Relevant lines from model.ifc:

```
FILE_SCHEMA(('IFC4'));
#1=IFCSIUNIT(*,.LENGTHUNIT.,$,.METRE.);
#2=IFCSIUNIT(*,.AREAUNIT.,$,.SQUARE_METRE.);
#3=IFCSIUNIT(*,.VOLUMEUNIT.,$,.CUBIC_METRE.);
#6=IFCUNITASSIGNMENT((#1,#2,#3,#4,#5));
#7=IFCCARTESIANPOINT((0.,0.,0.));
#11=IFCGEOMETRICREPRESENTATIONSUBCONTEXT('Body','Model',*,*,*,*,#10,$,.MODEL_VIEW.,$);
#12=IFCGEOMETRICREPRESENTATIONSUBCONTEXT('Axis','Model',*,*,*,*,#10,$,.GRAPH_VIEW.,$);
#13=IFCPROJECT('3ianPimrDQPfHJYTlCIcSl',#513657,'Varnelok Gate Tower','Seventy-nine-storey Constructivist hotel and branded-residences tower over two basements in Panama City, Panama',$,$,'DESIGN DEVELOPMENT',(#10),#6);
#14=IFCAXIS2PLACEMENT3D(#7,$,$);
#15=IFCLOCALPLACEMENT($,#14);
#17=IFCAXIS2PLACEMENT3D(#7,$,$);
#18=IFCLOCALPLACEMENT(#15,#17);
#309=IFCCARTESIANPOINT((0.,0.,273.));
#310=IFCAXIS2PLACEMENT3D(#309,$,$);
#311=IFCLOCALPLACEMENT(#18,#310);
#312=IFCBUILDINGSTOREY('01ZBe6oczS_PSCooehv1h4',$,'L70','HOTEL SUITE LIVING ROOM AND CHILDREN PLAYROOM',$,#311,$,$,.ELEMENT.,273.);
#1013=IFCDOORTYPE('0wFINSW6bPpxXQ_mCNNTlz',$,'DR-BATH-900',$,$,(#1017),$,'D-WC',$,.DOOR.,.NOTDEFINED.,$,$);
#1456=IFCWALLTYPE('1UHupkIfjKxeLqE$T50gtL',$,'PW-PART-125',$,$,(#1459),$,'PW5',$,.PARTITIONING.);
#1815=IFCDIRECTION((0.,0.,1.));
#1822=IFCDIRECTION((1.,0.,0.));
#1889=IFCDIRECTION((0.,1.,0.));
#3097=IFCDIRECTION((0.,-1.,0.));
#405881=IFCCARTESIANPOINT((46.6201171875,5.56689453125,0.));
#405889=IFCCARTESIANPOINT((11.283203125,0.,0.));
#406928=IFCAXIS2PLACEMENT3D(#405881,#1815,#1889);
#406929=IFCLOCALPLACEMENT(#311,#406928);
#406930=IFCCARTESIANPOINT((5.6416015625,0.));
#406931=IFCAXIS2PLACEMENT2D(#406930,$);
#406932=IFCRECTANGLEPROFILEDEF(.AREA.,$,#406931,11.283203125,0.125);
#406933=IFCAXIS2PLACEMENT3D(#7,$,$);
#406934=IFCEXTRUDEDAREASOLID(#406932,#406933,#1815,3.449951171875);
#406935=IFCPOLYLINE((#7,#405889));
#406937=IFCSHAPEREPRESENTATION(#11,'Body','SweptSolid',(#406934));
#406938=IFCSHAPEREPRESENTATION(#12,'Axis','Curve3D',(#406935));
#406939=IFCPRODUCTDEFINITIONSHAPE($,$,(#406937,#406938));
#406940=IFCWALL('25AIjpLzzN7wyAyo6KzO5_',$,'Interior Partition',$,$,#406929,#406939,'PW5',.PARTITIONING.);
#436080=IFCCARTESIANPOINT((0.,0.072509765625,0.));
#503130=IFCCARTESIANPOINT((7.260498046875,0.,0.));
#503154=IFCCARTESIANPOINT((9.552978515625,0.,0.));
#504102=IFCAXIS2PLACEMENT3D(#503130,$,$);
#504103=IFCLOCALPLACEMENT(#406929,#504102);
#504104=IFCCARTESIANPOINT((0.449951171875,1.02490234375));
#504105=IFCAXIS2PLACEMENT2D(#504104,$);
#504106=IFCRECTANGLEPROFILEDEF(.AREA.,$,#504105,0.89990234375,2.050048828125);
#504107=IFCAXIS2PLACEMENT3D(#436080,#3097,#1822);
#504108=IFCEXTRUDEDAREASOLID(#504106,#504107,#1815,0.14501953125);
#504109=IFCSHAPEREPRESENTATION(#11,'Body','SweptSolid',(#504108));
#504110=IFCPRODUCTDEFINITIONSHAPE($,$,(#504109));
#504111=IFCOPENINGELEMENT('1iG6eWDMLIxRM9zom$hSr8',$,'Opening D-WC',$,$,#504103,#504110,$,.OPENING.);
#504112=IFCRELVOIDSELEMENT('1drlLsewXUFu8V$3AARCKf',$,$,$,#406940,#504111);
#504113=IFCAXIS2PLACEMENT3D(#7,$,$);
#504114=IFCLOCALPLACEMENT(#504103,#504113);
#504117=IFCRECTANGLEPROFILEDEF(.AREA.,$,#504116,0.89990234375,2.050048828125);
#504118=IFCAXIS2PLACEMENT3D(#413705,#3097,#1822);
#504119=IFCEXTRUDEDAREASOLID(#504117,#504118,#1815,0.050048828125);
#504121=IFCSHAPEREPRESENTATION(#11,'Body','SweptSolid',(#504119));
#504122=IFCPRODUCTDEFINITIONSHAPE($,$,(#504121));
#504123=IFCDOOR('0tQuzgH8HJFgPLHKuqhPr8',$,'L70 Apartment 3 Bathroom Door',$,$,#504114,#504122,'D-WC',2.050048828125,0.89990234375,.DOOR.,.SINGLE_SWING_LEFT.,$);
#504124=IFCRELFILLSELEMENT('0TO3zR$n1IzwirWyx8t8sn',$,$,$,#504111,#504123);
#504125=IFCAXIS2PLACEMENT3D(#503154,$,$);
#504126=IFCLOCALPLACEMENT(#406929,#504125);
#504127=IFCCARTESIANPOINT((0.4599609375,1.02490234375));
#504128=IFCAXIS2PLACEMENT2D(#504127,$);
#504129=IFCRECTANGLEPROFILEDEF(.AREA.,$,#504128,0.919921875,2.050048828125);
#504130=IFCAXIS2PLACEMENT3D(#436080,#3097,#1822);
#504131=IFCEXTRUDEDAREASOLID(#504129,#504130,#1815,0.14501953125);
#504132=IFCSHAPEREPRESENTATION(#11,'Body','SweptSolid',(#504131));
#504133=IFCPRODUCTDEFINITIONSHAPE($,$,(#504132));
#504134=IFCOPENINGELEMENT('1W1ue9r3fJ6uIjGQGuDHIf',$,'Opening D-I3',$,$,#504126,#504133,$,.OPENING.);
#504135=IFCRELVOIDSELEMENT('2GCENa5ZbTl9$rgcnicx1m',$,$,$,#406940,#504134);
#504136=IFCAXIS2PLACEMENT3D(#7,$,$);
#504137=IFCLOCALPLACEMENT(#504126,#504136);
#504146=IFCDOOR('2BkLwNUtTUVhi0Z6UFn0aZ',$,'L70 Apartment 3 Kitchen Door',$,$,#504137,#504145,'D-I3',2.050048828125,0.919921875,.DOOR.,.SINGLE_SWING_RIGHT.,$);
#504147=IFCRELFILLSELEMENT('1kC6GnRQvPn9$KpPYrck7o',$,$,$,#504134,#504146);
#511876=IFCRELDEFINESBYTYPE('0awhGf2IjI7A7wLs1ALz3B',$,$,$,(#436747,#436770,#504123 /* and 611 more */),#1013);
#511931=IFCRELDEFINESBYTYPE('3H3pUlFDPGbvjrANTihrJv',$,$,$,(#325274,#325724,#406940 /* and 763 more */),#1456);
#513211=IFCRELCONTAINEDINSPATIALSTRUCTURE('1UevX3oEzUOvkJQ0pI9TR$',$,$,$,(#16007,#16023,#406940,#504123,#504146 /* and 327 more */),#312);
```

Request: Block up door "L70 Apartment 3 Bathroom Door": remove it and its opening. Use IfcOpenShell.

```python
import ifcopenshell
import ifcopenshell.api.feature
import ifcopenshell.api.root
import ifcopenshell.geom
import ifcopenshell.util.shape

model = ifcopenshell.open("model.ifc")
settings = ifcopenshell.geom.settings()


def volume(element):
    """Net volume in cubic metres, openings subtracted."""
    shape = ifcopenshell.geom.create_shape(settings, element)
    return ifcopenshell.util.shape.get_volume(shape.geometry)


door = model.by_guid("0tQuzgH8HJFgPLHKuqhPr8")
opening = door.FillsVoids[0].RelatingOpeningElement
wall = opening.VoidsElements[0].RelatingBuildingElement
before = volume(wall)

ifcopenshell.api.root.remove_product(model, product=door)
ifcopenshell.api.feature.remove_feature(model, feature=opening)

after = volume(wall)

print(f"wall volume {before:.3f} -> {after:.3f} m3")

model.write("model-out.ifc")
```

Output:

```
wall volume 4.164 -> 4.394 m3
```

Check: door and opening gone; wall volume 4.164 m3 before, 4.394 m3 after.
